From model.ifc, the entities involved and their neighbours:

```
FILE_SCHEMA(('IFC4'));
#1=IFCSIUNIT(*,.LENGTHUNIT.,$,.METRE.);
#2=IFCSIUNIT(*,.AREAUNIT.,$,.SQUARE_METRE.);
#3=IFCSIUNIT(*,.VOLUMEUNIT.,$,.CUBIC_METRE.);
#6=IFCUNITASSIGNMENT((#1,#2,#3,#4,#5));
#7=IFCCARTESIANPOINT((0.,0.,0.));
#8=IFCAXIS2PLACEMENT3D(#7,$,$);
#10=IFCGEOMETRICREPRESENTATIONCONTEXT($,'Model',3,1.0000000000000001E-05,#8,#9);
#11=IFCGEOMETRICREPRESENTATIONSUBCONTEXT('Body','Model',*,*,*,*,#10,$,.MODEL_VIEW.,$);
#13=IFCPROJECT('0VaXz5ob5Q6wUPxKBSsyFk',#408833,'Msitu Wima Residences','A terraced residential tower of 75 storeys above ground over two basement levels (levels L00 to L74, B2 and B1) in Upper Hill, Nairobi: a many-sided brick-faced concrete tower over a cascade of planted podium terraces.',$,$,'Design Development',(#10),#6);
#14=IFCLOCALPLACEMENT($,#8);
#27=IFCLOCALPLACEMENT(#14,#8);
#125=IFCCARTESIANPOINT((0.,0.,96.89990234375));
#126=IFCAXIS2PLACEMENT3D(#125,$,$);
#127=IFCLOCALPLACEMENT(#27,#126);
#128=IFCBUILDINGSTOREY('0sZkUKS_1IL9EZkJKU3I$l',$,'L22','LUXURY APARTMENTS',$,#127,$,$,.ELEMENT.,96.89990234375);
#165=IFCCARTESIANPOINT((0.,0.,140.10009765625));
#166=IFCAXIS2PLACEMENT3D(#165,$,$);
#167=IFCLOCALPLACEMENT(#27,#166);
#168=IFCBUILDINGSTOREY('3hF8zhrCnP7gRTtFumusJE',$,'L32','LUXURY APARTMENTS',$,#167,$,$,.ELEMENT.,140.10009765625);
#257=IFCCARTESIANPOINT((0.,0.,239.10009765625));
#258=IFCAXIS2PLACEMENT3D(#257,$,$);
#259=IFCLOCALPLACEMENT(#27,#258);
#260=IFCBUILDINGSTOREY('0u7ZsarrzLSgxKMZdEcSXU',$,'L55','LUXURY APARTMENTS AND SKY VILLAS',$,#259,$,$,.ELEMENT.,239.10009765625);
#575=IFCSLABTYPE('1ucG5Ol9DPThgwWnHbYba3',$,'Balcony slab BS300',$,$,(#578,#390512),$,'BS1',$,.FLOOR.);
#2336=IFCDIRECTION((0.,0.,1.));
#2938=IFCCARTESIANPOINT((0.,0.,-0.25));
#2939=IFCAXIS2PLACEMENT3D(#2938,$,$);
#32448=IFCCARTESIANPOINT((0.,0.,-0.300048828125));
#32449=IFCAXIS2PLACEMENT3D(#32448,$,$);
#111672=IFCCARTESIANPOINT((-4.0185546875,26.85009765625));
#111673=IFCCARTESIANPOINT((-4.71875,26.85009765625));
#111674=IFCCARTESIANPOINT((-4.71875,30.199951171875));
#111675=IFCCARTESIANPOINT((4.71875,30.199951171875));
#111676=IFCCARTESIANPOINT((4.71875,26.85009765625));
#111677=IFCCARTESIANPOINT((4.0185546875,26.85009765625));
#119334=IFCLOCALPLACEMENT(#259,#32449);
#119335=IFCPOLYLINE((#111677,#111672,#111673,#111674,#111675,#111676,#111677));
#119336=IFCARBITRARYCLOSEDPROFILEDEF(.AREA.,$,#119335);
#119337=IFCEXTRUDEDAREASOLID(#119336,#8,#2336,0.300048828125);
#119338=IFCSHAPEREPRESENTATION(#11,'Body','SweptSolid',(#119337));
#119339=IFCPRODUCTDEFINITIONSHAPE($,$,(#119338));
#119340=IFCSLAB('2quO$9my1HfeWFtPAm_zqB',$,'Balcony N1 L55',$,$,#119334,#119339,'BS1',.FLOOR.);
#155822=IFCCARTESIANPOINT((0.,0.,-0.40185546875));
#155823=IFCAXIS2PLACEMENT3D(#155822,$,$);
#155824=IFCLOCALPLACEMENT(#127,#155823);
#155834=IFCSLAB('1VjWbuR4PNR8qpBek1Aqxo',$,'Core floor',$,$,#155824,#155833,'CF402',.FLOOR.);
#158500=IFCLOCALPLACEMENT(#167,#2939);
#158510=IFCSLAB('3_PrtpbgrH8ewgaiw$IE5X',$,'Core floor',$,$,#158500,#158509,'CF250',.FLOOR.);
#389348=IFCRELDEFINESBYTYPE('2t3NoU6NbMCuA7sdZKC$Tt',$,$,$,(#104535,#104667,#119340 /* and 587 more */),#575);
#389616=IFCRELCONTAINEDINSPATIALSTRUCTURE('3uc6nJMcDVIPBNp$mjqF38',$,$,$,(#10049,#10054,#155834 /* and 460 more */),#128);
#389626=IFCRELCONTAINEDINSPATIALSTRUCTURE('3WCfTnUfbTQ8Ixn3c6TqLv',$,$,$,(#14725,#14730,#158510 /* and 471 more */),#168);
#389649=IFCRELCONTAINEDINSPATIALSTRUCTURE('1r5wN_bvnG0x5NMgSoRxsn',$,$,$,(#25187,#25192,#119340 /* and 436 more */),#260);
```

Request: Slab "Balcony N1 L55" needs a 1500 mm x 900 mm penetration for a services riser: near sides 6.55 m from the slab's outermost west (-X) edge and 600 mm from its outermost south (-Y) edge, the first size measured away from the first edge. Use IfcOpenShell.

```python
import numpy as np
import ifcopenshell
import ifcopenshell.api.feature
import ifcopenshell.api.geometry
import ifcopenshell.api.root
import ifcopenshell.geom
import ifcopenshell.util.placement
import ifcopenshell.util.representation
import ifcopenshell.util.shape
import ifcopenshell.util.unit

model = ifcopenshell.open("model.ifc")
unit_scale = ifcopenshell.util.unit.calculate_unit_scale(model)
settings = ifcopenshell.geom.settings()


def volume(element):
    """Net volume in cubic metres, openings subtracted."""
    shape = ifcopenshell.geom.create_shape(settings, element)
    return ifcopenshell.util.shape.get_volume(shape.geometry)


slab = model.by_guid("2quO$9my1HfeWFtPAm_zqB")
before = volume(slab)

# Extent in the slab's own axes, in metres. The edges named are its -X and -Y sides.
slab_shape = ifcopenshell.geom.create_shape(settings, slab)
vertices = ifcopenshell.util.shape.get_vertices(slab_shape.geometry)
x_min, y_min, bottom = vertices.min(axis=0)
top = vertices[:, 2].max()

opening = ifcopenshell.api.root.create_entity(model, ifc_class="IfcOpeningElement", name="Services riser opening", predefined_type="OPENING")
context = ifcopenshell.util.representation.get_context(model, "Model", "Body", "MODEL_VIEW")
width, depth = 1.5, 0.9
outline = [(0.0, 0.0), (width, 0.0), (width, depth), (0.0, depth), (0.0, 0.0)]
# Overshoot both faces by 50 mm so the cut is clean.
shape = ifcopenshell.api.geometry.add_slab_representation(
    model, context=context, depth=top - bottom + 0.1, polyline=outline
)
ifcopenshell.api.geometry.assign_representation(model, product=opening, representation=shape)

matrix = ifcopenshell.util.placement.get_local_placement(slab.ObjectPlacement)
matrix[:, 3] = matrix @ np.append(np.array([x_min + 6.55, y_min + 0.6, bottom - 0.05]) / unit_scale, 1.0)
ifcopenshell.api.geometry.edit_object_placement(model, product=opening, matrix=matrix, is_si=False)
ifcopenshell.api.feature.add_feature(model, feature=opening, element=slab)

after = volume(slab)

print(f"slab volume {before:.3f} -> {after:.3f} m3")

model.write("model_rev.ifc")
```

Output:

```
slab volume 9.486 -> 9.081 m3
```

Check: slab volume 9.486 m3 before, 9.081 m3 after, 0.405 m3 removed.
